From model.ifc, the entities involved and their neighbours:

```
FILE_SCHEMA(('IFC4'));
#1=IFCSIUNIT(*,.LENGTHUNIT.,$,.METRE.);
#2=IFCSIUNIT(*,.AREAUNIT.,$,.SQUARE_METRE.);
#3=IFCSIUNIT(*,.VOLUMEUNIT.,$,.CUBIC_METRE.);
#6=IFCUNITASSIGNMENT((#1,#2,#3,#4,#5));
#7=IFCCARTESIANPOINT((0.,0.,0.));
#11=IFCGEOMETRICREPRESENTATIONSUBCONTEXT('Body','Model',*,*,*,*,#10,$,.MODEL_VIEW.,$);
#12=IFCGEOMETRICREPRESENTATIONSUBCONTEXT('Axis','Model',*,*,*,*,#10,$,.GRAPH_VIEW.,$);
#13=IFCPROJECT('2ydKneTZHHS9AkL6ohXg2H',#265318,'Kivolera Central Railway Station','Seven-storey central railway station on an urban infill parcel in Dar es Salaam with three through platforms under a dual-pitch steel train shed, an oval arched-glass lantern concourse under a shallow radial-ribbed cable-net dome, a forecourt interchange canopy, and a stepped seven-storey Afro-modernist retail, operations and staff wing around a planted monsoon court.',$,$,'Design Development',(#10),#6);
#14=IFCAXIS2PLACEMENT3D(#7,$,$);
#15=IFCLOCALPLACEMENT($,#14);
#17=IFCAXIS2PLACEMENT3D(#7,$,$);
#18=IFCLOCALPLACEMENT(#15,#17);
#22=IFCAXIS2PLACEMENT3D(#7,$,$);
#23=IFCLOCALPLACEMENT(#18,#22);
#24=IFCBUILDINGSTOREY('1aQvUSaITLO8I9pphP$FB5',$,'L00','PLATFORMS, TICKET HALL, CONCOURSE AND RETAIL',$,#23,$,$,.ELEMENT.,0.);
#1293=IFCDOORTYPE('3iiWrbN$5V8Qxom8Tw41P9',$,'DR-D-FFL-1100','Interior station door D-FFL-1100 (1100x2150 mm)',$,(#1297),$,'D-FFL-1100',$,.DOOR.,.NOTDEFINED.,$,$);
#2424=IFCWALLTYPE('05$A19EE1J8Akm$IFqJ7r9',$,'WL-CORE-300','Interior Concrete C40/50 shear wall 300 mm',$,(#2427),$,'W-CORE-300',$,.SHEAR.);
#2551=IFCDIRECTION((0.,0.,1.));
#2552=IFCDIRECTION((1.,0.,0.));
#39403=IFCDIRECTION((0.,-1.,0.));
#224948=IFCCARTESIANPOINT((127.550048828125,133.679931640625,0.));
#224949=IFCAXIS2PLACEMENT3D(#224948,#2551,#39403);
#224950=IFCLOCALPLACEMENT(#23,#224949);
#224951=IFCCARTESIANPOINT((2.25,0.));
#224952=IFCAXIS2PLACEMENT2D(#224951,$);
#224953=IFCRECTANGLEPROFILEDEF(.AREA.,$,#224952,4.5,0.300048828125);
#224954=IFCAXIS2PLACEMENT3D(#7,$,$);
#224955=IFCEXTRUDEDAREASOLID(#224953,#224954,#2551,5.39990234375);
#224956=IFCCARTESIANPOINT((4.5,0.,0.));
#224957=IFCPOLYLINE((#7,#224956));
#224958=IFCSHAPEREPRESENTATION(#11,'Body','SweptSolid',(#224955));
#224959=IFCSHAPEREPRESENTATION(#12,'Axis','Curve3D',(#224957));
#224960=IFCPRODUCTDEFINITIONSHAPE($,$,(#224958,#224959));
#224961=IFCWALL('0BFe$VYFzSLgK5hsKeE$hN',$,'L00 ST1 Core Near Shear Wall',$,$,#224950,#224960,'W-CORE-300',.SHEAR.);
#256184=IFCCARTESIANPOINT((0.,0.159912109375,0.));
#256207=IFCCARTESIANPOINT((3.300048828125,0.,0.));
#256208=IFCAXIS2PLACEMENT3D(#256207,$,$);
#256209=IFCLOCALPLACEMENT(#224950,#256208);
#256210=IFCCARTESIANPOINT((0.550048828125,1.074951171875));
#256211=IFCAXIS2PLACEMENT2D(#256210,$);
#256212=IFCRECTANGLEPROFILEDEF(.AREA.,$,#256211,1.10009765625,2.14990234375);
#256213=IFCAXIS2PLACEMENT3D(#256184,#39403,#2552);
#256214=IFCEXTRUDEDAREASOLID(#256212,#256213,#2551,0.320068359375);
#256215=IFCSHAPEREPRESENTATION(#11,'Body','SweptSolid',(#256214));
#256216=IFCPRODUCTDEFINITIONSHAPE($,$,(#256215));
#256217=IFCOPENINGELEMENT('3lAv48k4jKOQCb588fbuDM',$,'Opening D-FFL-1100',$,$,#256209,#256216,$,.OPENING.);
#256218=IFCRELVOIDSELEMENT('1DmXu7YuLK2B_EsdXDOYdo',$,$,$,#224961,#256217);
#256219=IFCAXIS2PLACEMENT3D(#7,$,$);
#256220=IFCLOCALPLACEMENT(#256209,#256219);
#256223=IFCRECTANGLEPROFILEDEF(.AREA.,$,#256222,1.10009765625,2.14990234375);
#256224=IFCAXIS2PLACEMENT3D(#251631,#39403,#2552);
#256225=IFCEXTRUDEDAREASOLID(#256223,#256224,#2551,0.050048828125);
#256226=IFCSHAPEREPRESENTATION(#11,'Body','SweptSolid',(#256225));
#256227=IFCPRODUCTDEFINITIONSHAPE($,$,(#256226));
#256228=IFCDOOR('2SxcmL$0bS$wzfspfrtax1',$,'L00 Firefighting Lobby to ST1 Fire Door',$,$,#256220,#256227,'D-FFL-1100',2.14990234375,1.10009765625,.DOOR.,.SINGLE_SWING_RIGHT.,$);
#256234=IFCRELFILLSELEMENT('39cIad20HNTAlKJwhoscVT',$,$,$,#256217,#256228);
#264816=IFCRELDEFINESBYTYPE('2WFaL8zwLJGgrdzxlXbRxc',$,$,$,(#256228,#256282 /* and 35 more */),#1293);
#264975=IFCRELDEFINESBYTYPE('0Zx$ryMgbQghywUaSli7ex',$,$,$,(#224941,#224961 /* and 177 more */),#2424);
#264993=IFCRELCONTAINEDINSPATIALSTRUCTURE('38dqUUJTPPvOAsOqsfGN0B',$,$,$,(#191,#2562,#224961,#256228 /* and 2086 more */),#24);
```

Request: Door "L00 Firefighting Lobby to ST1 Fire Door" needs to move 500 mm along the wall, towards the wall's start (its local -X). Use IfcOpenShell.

```python
import ifcopenshell
import ifcopenshell.api.geometry
import ifcopenshell.util.placement
import ifcopenshell.util.unit

model = ifcopenshell.open("model.ifc")
unit_scale = ifcopenshell.util.unit.calculate_unit_scale(model)

door = model.by_guid("2SxcmL$0bS$wzfspfrtax1")
opening = door.FillsVoids[0].RelatingOpeningElement
wall = opening.VoidsElements[0].RelatingBuildingElement

wall_matrix = ifcopenshell.util.placement.get_local_placement(wall.ObjectPlacement)
shift = wall_matrix[:3, 0] * -0.5 / unit_scale
before = ifcopenshell.util.placement.get_local_placement(door.ObjectPlacement)[:3, 3].copy()

# The door is placed relative to its opening, so it follows when the opening moves.
matrix = ifcopenshell.util.placement.get_local_placement(opening.ObjectPlacement)
matrix[:3, 3] += shift
ifcopenshell.api.geometry.edit_object_placement(
    model, product=opening, matrix=matrix, is_si=False, should_transform_children=True
)

after = ifcopenshell.util.placement.get_local_placement(door.ObjectPlacement)[:3, 3]
print("door moved by", (after - before).round(3) + 0.0)

model.write("model_rev.ifc")
```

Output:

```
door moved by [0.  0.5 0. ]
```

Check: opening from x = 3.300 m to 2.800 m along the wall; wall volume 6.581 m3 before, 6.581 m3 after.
